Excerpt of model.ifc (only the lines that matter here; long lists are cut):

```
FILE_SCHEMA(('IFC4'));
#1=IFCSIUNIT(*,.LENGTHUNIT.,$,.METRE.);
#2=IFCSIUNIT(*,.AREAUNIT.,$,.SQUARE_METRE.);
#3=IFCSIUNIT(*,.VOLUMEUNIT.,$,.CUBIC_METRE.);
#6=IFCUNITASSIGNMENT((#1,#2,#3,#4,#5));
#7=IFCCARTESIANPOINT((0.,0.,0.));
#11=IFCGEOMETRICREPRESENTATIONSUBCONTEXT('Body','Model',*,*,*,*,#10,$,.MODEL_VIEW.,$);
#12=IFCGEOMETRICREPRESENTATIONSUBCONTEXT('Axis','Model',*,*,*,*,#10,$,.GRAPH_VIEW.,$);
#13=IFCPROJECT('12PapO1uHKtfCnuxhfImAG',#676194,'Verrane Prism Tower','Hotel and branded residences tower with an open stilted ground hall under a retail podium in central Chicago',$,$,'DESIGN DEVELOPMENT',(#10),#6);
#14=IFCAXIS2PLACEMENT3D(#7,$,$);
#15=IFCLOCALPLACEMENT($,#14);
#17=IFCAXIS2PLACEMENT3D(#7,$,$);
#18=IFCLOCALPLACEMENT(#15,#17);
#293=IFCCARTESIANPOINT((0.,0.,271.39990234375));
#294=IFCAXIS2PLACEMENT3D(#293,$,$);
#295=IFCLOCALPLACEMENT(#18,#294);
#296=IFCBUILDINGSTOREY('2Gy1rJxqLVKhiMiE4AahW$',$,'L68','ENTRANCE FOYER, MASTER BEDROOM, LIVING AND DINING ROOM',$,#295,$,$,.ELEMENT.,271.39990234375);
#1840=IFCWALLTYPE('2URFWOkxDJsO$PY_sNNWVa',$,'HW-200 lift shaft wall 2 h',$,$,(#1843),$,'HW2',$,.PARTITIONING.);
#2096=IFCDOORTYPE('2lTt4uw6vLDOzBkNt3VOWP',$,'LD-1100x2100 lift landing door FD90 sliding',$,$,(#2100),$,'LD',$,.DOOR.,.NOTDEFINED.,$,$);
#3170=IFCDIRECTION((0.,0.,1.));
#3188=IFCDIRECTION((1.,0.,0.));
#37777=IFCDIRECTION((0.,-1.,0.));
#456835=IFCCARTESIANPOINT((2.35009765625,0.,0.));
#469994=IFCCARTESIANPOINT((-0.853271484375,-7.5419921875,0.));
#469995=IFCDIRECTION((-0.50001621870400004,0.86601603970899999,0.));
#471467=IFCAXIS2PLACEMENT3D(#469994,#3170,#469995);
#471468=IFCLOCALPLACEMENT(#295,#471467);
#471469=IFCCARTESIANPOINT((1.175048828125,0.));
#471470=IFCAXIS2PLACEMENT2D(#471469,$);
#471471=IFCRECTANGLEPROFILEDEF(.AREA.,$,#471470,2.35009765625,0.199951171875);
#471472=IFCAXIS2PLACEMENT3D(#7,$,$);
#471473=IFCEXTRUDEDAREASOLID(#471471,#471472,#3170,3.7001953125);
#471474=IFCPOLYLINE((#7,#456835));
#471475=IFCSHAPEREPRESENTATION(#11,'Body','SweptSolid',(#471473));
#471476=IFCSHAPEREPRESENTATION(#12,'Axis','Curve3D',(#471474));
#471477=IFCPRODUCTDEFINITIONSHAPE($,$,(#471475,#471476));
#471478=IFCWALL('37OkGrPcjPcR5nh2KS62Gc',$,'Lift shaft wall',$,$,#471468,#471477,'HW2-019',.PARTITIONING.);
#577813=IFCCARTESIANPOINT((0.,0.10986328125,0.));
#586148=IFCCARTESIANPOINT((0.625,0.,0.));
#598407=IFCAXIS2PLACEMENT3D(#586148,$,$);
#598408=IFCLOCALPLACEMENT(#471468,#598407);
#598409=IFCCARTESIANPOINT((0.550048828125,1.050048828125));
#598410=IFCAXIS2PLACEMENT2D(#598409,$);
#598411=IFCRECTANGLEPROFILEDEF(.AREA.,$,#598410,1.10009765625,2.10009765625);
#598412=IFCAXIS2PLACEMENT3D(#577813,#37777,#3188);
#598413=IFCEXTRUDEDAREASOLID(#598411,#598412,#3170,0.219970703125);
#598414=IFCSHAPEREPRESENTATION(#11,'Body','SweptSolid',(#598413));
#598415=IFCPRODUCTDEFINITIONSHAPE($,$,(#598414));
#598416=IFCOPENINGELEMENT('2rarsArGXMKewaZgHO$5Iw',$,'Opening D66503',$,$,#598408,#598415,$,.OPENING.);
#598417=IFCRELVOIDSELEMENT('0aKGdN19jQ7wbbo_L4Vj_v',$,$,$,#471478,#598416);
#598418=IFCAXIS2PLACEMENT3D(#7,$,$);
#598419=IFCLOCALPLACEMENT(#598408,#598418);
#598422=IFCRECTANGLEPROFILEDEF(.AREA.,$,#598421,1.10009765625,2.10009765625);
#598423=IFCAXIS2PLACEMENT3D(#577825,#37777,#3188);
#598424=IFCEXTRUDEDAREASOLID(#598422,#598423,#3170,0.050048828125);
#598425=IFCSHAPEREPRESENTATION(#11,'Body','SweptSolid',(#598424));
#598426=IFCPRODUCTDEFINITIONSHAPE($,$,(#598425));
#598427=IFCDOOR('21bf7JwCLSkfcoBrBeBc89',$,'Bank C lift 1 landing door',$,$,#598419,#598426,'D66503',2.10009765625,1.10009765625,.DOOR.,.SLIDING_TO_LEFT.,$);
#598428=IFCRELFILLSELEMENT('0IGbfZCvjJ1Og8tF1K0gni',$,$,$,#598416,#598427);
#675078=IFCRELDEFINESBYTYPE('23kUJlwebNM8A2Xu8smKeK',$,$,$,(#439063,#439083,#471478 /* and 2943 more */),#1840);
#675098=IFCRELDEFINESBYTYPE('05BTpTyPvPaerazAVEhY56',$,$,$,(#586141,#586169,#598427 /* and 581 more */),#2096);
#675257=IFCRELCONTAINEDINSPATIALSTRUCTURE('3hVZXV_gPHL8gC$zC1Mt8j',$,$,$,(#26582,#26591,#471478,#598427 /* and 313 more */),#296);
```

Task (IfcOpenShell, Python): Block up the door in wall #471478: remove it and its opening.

```python
import ifcopenshell
import ifcopenshell.api.feature
import ifcopenshell.api.root
import ifcopenshell.geom
import ifcopenshell.util.shape

model = ifcopenshell.open("model.ifc")
settings = ifcopenshell.geom.settings()


def volume(element):
    """Net volume in cubic metres, openings subtracted."""
    shape = ifcopenshell.geom.create_shape(settings, element)
    return ifcopenshell.util.shape.get_volume(shape.geometry)


door = model.by_id(598427)
opening = door.FillsVoids[0].RelatingOpeningElement
wall = opening.VoidsElements[0].RelatingBuildingElement
before = volume(wall)

ifcopenshell.api.root.remove_product(model, product=door)
ifcopenshell.api.feature.remove_feature(model, feature=opening)

after = volume(wall)

print(f"wall volume {before:.3f} -> {after:.3f} m3")

model.write("model_edited.ifc")
```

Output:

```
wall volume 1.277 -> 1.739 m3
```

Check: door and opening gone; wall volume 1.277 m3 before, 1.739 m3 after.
